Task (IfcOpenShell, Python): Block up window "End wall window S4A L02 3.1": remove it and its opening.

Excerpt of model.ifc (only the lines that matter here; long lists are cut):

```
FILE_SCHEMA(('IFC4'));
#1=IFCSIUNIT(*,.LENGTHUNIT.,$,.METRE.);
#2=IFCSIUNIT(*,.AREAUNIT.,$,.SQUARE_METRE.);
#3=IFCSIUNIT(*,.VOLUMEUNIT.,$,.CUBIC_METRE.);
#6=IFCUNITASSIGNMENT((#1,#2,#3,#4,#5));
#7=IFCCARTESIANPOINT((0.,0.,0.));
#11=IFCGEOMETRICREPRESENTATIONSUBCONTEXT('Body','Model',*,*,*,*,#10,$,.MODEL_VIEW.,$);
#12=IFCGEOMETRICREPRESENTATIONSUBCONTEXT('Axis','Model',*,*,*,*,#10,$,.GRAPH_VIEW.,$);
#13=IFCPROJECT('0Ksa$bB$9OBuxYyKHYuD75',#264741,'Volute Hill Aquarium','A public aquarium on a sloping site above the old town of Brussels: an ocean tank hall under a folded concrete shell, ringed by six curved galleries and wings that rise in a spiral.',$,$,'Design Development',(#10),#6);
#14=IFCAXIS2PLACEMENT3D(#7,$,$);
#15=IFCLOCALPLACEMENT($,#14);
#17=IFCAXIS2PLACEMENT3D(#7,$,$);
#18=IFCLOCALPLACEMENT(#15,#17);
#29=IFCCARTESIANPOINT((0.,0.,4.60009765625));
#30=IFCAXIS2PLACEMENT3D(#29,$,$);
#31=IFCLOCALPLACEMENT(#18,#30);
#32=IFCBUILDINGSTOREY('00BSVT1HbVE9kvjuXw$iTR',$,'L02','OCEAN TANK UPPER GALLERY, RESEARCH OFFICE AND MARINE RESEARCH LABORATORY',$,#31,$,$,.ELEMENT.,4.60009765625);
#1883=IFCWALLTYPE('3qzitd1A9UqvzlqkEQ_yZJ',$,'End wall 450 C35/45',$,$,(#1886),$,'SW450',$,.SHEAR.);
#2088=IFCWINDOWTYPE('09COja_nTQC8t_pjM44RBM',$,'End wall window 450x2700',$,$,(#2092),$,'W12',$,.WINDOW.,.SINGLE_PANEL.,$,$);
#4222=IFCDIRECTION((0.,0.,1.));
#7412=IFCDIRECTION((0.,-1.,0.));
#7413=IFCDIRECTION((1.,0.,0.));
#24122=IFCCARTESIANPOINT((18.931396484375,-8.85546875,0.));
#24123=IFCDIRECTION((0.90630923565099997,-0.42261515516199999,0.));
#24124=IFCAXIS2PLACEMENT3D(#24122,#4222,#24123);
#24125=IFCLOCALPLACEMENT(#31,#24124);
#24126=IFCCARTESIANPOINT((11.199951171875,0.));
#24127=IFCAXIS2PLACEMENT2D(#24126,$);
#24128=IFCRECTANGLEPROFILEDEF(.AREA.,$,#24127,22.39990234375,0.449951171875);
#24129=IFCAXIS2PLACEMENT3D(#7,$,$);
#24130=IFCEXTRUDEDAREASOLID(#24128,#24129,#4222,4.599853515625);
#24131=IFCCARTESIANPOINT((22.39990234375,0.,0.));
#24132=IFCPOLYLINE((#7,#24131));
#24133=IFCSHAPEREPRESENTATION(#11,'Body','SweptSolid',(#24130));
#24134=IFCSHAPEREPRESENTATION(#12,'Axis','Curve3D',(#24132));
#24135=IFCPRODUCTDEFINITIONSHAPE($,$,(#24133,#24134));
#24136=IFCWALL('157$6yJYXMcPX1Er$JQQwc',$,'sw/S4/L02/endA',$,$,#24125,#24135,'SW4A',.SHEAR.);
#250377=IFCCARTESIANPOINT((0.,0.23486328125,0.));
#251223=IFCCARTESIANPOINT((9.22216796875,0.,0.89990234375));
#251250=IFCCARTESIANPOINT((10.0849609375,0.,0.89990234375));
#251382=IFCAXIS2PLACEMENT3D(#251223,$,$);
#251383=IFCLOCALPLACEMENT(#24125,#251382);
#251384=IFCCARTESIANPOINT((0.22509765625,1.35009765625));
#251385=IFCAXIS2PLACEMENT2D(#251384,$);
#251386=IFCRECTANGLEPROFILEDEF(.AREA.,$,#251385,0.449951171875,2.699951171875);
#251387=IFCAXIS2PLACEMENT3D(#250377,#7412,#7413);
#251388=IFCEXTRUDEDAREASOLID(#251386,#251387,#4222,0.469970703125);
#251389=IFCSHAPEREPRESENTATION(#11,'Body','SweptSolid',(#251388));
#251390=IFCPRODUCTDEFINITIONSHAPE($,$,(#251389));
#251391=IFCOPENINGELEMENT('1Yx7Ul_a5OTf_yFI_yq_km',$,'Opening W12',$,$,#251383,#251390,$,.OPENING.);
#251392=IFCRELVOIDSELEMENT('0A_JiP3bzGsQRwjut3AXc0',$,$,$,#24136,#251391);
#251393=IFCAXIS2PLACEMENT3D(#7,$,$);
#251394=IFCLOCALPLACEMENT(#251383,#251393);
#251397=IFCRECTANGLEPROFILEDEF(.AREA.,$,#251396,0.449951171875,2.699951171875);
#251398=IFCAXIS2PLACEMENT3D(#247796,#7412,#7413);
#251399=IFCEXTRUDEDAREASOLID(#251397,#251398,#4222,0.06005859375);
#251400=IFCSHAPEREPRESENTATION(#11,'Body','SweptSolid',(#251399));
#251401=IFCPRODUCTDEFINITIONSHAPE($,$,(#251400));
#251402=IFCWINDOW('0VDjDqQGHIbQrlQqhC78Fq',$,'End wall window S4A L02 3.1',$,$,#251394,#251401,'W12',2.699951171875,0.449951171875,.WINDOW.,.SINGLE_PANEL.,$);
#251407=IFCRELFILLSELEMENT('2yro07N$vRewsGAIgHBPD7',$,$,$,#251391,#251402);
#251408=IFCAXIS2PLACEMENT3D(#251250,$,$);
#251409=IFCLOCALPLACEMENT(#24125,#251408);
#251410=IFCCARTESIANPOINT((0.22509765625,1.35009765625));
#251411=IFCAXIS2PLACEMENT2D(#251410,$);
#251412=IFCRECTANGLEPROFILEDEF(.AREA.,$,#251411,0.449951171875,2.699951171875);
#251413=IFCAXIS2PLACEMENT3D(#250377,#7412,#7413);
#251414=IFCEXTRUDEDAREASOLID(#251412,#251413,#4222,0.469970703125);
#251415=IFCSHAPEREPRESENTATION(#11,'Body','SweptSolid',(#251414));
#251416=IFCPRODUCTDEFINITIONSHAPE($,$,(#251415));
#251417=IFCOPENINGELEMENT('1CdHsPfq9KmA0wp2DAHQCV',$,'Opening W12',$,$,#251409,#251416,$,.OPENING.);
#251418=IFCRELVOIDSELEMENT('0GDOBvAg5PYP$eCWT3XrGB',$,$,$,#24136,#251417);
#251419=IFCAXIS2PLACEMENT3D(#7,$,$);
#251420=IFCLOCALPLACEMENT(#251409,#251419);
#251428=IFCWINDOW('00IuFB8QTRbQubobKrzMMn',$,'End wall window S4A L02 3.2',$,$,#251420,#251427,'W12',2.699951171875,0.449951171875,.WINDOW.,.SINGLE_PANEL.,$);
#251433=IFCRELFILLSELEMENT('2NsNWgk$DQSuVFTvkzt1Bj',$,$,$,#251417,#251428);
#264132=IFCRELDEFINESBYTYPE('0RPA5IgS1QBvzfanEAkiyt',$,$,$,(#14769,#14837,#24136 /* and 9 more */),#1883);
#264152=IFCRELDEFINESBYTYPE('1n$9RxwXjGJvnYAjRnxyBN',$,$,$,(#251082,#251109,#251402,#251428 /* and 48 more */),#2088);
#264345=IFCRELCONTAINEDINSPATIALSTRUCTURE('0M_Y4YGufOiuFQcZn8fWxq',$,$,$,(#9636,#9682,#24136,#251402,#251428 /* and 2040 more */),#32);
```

```python
import ifcopenshell
import ifcopenshell.api.feature
import ifcopenshell.api.root
import ifcopenshell.geom
import ifcopenshell.util.shape

model = ifcopenshell.open("model.ifc")
settings = ifcopenshell.geom.settings()


def volume(element):
    """Net volume in cubic metres, openings subtracted."""
    shape = ifcopenshell.geom.create_shape(settings, element)
    return ifcopenshell.util.shape.get_volume(shape.geometry)


window = model.by_guid("0VDjDqQGHIbQrlQqhC78Fq")
opening = window.FillsVoids[0].RelatingOpeningElement
wall = opening.VoidsElements[0].RelatingBuildingElement
before = volume(wall)

ifcopenshell.api.root.remove_product(model, product=window)
ifcopenshell.api.feature.remove_feature(model, feature=opening)

after = volume(wall)

print(f"wall volume {before:.3f} -> {after:.3f} m3")

model.write("model_v2.ifc")
```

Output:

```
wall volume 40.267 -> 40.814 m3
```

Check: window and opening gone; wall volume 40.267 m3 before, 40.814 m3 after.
